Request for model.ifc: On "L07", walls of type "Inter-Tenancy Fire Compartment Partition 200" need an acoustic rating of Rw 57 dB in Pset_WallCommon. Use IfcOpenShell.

First a look at what the model holds.

```python
import ifcopenshell
import ifcopenshell.util.element

model = ifcopenshell.open("model.ifc")
print(model.schema)
storey = next(s for s in model.by_type("IfcBuildingStorey") if s.Name == "L07")
walls = [e for e in ifcopenshell.util.element.get_decomposition(storey) if e.is_a("IfcWall")]
seen = {}
for e in walls:
    element_type = ifcopenshell.util.element.get_type(e)
    key = (element_type.Name if element_type != e and element_type else None, ifcopenshell.util.element.get_pset(e, "Pset_WallCommon", "AcousticRating"))
    seen[key] = seen.get(key, 0) + 1
for (name, value), count in sorted(seen.items(), key=str):
    print(count, "x", name, "|", value)
```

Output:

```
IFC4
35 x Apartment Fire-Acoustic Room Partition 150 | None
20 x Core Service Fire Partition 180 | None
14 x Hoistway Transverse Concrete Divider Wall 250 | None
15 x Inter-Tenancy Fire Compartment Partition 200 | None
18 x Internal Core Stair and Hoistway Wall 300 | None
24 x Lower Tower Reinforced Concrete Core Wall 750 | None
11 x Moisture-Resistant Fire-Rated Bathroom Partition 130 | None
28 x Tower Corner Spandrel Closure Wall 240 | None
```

```python
import ifcopenshell
import ifcopenshell.api.pset
import ifcopenshell.util.element

model = ifcopenshell.open("model.ifc")

storey = next(s for s in model.by_type("IfcBuildingStorey") if s.Name == "L07")
walls = [e for e in ifcopenshell.util.element.get_decomposition(storey) if e.is_a("IfcWall")]

count = 0
for e in walls:
    element_type = ifcopenshell.util.element.get_type(e)
    if element_type in (None, e) or element_type.Name != "Inter-Tenancy Fire Compartment Partition 200":
        continue
    found = ifcopenshell.util.element.get_pset(e, "Pset_WallCommon", should_inherit=False)
    if found:
        pset = model.by_id(found["id"])
        if len(ifcopenshell.util.element.get_elements_by_pset(pset)) > 1:
            pset = ifcopenshell.api.pset.unshare_pset(model, products=[e], pset=pset)[0]
    else:
        pset = ifcopenshell.api.pset.add_pset(model, product=e, name="Pset_WallCommon")
    ifcopenshell.api.pset.edit_pset(model, pset=pset, properties={"AcousticRating": "Rw 57 dB"})
    count += 1

print(count, "walls updated")

model.write("model_rev.ifc")
```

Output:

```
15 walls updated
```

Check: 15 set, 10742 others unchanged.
